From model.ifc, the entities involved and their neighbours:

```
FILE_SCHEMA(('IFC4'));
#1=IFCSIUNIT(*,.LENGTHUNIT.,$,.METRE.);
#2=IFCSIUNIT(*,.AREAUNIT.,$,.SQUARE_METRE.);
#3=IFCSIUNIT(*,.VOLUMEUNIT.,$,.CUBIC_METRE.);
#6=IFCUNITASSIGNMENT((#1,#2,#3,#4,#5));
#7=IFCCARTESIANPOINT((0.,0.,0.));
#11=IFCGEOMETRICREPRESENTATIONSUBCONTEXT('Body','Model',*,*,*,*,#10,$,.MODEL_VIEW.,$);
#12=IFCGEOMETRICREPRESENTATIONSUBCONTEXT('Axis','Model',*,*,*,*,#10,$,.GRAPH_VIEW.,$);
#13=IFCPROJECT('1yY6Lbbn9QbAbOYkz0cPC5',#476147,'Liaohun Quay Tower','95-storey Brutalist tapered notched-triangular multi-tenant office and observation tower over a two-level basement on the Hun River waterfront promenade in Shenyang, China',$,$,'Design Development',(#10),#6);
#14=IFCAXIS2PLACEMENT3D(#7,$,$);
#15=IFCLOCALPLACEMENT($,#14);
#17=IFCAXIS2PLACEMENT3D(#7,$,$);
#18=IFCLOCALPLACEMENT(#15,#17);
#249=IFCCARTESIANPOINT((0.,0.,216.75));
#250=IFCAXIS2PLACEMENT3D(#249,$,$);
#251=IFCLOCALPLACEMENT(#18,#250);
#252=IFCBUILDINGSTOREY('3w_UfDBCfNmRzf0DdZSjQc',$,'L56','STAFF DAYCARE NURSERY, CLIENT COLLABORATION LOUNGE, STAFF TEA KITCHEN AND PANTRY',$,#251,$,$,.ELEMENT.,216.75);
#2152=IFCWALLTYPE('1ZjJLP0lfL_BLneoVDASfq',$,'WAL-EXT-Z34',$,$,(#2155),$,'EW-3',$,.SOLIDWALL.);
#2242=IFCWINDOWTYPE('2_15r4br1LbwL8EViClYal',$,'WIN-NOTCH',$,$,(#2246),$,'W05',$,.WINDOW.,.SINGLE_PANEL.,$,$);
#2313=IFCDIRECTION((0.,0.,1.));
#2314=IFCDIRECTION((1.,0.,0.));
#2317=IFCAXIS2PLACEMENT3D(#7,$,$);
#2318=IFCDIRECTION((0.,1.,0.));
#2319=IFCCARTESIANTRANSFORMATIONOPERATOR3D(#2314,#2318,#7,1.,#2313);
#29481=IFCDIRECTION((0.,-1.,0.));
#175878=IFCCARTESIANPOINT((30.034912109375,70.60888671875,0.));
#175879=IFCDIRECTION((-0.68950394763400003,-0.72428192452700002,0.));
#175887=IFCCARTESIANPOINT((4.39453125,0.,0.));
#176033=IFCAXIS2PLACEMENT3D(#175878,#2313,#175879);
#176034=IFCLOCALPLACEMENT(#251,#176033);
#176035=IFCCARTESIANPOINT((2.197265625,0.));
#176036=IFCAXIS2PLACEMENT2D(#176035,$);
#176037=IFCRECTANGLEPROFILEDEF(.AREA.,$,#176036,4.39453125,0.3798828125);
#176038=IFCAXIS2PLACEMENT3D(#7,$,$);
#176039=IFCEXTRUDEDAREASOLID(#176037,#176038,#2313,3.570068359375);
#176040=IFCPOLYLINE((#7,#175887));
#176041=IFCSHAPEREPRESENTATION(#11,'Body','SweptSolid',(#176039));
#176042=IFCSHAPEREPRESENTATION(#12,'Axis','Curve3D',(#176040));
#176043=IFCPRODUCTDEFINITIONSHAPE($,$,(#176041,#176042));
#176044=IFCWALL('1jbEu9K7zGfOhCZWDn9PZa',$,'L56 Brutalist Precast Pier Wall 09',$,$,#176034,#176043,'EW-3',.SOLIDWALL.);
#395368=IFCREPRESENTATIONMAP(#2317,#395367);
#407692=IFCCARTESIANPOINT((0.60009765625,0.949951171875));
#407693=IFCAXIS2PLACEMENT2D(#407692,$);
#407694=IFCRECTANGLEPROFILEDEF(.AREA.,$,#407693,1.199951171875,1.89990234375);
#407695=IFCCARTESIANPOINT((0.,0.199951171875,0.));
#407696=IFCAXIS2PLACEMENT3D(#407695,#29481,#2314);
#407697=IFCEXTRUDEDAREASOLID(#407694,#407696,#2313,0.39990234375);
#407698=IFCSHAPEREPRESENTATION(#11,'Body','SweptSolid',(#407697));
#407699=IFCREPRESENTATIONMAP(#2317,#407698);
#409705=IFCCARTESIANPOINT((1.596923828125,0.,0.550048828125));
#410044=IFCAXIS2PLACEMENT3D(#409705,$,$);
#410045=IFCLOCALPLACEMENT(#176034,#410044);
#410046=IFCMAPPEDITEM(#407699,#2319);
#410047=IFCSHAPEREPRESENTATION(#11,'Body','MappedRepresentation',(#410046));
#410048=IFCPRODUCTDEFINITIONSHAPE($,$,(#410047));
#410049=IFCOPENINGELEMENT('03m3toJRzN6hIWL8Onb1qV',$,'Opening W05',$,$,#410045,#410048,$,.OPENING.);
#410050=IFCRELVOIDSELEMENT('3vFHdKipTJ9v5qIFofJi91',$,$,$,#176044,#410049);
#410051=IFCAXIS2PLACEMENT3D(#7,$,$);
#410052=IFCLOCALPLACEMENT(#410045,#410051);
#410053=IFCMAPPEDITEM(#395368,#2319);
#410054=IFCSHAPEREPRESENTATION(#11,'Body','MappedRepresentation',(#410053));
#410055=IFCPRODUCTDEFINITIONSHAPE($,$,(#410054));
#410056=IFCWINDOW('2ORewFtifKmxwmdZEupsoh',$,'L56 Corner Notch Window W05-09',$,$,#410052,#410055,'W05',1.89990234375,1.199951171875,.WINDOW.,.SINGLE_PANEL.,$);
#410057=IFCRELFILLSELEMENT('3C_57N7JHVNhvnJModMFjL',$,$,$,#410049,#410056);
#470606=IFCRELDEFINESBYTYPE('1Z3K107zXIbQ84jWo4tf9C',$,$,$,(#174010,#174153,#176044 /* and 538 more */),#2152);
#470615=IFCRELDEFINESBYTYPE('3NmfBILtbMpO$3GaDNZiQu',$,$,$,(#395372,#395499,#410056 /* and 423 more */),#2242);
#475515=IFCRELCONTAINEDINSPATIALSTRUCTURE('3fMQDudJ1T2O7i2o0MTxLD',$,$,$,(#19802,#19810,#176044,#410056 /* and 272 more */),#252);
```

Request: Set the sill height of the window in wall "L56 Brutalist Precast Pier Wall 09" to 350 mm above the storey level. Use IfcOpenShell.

```python
import numpy as np
import ifcopenshell
import ifcopenshell.api.geometry
import ifcopenshell.geom
import ifcopenshell.util.element
import ifcopenshell.util.placement
import ifcopenshell.util.shape
import ifcopenshell.util.unit

model = ifcopenshell.open("model.ifc")
unit_scale = ifcopenshell.util.unit.calculate_unit_scale(model)

window = model.by_guid("2ORewFtifKmxwmdZEupsoh")
opening = window.FillsVoids[0].RelatingOpeningElement
storey = ifcopenshell.util.element.get_container(window, ifc_class="IfcBuildingStorey")
level = ifcopenshell.util.placement.get_local_placement(storey.ObjectPlacement)[2, 3]

# The opening's origin need not be at the sill, so measure its lowest point.
shape = ifcopenshell.geom.create_shape(ifcopenshell.geom.settings(), opening)
bottom = ifcopenshell.util.shape.get_shape_bottom_elevation(shape, shape.geometry) / unit_scale
dz = level + 0.35 / unit_scale - bottom

shift = np.array([0.0, 0.0, dz])
# The window is placed relative to its opening, so it follows when the opening moves.
matrix = ifcopenshell.util.placement.get_local_placement(opening.ObjectPlacement)
matrix[:3, 3] += shift
ifcopenshell.api.geometry.edit_object_placement(
    model, product=opening, matrix=matrix, is_si=False, should_transform_children=True
)

print(f"moved by {dz * unit_scale:+.3f} m")

model.write("model_edited.ifc")
```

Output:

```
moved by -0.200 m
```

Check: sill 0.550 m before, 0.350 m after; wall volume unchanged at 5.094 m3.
